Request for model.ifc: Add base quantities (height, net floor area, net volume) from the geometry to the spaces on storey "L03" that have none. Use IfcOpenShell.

First a look at what the model holds.

```python
import ifcopenshell
import ifcopenshell.util.element
import ifcopenshell.util.unit

model = ifcopenshell.open("model.ifc")
print(model.schema)
for unit_type in ("LENGTHUNIT", "AREAUNIT", "VOLUMEUNIT"):
    print(unit_type, ifcopenshell.util.unit.calculate_unit_scale(model, unit_type))
storey = next(s for s in model.by_type("IfcBuildingStorey") if s.Name == "L03")
spaces = [e for e in ifcopenshell.util.element.get_decomposition(storey) if e.is_a("IfcSpace")]
for e in sorted(spaces, key=lambda e: e.id()):
    print(e.id(), e.is_a(), e.Name, list(ifcopenshell.util.element.get_psets(e, qtos_only=True)), sep=" | ")
```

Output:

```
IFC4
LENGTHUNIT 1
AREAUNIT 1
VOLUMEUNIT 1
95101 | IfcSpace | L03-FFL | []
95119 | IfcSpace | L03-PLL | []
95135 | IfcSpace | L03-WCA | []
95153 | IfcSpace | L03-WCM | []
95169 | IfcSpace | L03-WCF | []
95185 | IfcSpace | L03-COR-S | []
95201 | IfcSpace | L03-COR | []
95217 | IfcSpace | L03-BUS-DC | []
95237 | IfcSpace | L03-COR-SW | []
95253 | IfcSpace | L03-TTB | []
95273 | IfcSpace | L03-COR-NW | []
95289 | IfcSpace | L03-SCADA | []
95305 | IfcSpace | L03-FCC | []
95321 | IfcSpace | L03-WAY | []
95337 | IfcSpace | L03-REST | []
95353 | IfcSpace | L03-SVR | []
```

```python
import ifcopenshell
import ifcopenshell.api.pset
import ifcopenshell.geom
import ifcopenshell.util.element
import ifcopenshell.util.shape
import ifcopenshell.util.unit

model = ifcopenshell.open("model.ifc")
unit_scale = ifcopenshell.util.unit.calculate_unit_scale(model)
area_scale = ifcopenshell.util.unit.calculate_unit_scale(model, "AREAUNIT")
volume_scale = ifcopenshell.util.unit.calculate_unit_scale(model, "VOLUMEUNIT")
settings = ifcopenshell.geom.settings()

storey = next(s for s in model.by_type("IfcBuildingStorey") if s.Name == "L03")
spaces = [e for e in ifcopenshell.util.element.get_decomposition(storey) if e.is_a("IfcSpace")]

for e in sorted(spaces, key=lambda e: e.id()):
    if ifcopenshell.util.element.get_psets(e, qtos_only=True, should_inherit=False):
        continue
    # Geometry comes back in metres, in the element's own axes.
    shape = ifcopenshell.geom.create_shape(settings, e)
    values = {
        "Height": ifcopenshell.util.shape.get_z(shape.geometry) / unit_scale,
        "NetFloorArea": ifcopenshell.util.shape.get_footprint_area(shape.geometry) / area_scale,
        "NetVolume": ifcopenshell.util.shape.get_volume(shape.geometry) / volume_scale,
    }
    qto = ifcopenshell.api.pset.add_qto(model, product=e, name="Qto_SpaceBaseQuantities")
    ifcopenshell.api.pset.edit_qto(model, qto=qto, properties=values)
    print(e.id(), {k: round(v, 3) for k, v in values.items()})

model.write("model_rev.ifc")
```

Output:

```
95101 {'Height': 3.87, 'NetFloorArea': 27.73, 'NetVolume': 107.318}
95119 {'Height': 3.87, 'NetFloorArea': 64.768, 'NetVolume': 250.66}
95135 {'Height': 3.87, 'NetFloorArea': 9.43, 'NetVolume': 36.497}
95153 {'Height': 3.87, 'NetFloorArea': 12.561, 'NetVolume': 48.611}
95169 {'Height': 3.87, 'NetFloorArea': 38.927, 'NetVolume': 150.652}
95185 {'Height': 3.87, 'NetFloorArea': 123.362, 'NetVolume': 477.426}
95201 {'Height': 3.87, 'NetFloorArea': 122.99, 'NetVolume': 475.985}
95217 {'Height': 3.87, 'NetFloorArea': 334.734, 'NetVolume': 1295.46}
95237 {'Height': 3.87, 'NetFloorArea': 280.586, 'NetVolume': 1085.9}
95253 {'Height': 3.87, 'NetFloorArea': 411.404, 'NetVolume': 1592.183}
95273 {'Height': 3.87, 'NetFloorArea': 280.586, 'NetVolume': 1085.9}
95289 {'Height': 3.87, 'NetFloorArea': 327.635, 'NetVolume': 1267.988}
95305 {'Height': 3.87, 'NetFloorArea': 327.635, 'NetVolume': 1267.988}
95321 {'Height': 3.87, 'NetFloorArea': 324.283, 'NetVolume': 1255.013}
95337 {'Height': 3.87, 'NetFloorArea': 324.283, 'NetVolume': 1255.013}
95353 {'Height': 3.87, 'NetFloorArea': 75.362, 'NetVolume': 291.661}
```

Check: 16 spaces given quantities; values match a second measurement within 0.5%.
